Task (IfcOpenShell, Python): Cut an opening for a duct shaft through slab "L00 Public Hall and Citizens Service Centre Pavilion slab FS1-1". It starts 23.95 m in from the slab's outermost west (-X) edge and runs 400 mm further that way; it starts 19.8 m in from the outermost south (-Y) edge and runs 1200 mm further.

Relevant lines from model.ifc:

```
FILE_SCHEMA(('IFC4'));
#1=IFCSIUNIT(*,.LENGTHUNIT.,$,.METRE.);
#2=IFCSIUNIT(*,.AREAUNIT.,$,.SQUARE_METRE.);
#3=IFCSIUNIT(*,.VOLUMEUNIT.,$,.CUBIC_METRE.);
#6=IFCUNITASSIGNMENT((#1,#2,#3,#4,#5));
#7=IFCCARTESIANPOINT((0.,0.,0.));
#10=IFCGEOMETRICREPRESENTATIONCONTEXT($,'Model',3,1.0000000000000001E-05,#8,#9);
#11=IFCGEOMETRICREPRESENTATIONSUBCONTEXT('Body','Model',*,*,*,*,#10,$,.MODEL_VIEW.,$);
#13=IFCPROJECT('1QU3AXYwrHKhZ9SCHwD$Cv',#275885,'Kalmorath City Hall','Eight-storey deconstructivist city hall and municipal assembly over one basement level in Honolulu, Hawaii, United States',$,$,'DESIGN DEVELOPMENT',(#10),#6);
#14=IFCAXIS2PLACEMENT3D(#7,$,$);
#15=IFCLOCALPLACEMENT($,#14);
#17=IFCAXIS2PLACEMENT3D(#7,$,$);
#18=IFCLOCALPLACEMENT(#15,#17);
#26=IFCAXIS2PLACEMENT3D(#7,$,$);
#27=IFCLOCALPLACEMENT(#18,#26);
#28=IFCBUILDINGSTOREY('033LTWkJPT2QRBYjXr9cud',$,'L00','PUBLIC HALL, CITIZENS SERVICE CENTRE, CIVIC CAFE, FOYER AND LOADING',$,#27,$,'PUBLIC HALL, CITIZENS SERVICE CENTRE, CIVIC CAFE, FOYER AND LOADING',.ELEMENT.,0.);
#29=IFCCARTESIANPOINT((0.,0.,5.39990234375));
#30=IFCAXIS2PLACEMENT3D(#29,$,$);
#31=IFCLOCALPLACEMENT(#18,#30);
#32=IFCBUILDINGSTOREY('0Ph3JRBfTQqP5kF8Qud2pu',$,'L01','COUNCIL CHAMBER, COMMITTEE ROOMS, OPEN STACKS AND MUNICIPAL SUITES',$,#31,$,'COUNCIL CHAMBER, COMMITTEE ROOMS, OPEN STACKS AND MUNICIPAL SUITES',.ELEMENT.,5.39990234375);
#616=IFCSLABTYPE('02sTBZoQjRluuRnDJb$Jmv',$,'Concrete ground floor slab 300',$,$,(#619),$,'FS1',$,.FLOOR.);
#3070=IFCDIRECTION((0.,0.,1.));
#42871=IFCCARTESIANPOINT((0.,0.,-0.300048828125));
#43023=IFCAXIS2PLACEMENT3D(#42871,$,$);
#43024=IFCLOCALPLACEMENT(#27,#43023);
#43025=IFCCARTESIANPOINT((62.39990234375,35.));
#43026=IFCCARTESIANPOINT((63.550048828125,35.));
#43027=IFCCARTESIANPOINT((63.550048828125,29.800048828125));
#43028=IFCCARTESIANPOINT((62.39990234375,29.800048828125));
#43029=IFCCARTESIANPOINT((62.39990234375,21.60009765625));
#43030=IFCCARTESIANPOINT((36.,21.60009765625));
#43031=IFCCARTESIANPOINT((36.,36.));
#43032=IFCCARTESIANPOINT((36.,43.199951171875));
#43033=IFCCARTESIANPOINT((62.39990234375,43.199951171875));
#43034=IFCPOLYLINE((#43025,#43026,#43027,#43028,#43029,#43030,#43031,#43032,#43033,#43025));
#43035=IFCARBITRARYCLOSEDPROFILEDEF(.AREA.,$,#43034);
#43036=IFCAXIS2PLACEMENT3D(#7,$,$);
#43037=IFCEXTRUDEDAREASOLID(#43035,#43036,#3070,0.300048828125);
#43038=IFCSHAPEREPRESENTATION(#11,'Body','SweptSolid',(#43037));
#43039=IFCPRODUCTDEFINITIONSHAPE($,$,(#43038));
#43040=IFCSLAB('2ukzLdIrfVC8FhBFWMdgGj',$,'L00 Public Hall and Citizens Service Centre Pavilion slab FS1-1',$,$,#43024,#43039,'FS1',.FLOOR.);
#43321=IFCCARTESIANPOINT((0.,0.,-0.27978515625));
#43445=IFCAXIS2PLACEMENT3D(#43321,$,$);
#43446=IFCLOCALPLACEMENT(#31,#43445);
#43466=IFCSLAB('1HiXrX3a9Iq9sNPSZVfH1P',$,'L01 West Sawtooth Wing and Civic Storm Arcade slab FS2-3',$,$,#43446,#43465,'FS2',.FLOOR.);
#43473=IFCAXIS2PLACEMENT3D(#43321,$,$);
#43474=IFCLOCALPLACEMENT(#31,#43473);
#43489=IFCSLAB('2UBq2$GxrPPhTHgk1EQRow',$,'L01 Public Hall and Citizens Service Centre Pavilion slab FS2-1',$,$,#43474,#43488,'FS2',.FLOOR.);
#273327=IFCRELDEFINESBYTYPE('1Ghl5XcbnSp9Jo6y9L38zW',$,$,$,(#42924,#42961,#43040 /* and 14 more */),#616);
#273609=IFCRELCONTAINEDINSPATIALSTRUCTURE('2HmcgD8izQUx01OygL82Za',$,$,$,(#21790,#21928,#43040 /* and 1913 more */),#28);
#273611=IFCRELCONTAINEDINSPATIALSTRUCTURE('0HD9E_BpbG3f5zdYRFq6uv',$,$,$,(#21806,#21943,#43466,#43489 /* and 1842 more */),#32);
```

```python
import numpy as np
import ifcopenshell
import ifcopenshell.api.feature
import ifcopenshell.api.geometry
import ifcopenshell.api.root
import ifcopenshell.geom
import ifcopenshell.util.placement
import ifcopenshell.util.representation
import ifcopenshell.util.shape
import ifcopenshell.util.unit

model = ifcopenshell.open("model.ifc")
unit_scale = ifcopenshell.util.unit.calculate_unit_scale(model)
settings = ifcopenshell.geom.settings()


def volume(element):
    """Net volume in cubic metres, openings subtracted."""
    shape = ifcopenshell.geom.create_shape(settings, element)
    return ifcopenshell.util.shape.get_volume(shape.geometry)


slab = model.by_guid("2ukzLdIrfVC8FhBFWMdgGj")
before = volume(slab)

# Extent in the slab's own axes, in metres. The edges named are its -X and -Y sides.
slab_shape = ifcopenshell.geom.create_shape(settings, slab)
vertices = ifcopenshell.util.shape.get_vertices(slab_shape.geometry)
x_min, y_min, bottom = vertices.min(axis=0)
top = vertices[:, 2].max()

opening = ifcopenshell.api.root.create_entity(model, ifc_class="IfcOpeningElement", name="Duct shaft opening", predefined_type="OPENING")
context = ifcopenshell.util.representation.get_context(model, "Model", "Body", "MODEL_VIEW")
width, depth = 0.4, 1.2
outline = [(0.0, 0.0), (width, 0.0), (width, depth), (0.0, depth), (0.0, 0.0)]
# Overshoot both faces by 50 mm so the cut is clean.
shape = ifcopenshell.api.geometry.add_slab_representation(
    model, context=context, depth=top - bottom + 0.1, polyline=outline
)
ifcopenshell.api.geometry.assign_representation(model, product=opening, representation=shape)

matrix = ifcopenshell.util.placement.get_local_placement(slab.ObjectPlacement)
matrix[:, 3] = matrix @ np.append(np.array([x_min + 23.95, y_min + 19.8, bottom - 0.05]) / unit_scale, 1.0)
ifcopenshell.api.geometry.edit_object_placement(model, product=opening, matrix=matrix, is_si=False)
ifcopenshell.api.feature.add_feature(model, feature=opening, element=slab)

after = volume(slab)

print(f"slab volume {before:.3f} -> {after:.3f} m3")

model.write("model_edited.ifc")
```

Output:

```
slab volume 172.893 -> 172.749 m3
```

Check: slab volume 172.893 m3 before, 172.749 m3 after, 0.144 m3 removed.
